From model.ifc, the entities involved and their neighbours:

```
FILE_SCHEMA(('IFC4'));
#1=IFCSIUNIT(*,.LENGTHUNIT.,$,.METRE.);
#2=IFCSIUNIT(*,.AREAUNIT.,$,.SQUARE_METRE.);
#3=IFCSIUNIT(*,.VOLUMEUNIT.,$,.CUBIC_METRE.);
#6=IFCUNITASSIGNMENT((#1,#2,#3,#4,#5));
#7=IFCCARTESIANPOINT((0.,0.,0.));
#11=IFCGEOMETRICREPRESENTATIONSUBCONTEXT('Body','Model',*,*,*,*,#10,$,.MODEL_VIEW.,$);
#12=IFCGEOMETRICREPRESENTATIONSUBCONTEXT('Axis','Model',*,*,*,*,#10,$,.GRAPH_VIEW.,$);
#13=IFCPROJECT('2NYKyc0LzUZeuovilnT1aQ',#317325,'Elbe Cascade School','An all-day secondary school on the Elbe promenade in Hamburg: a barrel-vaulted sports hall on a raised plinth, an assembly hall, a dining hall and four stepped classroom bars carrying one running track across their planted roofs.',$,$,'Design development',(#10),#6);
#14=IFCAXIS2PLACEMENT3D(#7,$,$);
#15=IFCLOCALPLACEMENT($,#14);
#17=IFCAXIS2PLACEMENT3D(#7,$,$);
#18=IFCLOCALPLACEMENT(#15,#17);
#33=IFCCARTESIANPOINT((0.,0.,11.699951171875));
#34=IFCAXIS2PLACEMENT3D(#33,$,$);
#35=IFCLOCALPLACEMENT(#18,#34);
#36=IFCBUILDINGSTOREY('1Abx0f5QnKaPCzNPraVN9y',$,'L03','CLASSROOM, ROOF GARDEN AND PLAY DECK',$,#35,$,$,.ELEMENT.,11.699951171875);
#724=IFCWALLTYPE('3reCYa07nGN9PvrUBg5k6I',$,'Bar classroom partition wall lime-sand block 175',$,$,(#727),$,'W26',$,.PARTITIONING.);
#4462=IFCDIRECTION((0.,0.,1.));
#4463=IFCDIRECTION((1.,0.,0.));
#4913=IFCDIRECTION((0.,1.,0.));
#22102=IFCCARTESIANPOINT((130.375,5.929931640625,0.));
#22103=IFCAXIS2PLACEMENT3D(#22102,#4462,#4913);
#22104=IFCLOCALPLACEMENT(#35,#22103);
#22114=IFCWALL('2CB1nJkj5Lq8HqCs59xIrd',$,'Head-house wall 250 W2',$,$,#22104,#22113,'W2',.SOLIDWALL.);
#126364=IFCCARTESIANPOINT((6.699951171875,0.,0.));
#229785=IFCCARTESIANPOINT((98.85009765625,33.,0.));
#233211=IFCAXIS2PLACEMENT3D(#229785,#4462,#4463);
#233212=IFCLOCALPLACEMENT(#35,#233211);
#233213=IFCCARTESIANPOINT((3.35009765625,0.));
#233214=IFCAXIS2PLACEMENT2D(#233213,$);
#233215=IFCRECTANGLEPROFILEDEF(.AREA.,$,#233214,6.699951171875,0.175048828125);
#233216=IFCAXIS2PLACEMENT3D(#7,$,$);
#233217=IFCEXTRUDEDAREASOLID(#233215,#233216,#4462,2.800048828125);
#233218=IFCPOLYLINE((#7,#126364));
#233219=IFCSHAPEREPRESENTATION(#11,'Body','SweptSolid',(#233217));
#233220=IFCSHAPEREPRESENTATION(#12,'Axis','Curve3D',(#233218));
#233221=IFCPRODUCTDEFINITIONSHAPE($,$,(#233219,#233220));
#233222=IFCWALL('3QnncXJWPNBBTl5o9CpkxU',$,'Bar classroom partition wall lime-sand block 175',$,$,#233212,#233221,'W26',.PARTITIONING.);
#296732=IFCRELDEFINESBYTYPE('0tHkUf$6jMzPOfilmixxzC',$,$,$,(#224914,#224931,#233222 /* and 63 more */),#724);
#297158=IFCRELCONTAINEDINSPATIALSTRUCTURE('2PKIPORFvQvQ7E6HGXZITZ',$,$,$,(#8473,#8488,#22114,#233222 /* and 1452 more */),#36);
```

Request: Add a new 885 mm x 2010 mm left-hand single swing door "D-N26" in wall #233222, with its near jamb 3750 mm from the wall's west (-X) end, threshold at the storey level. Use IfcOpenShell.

```python
import numpy as np
import ifcopenshell
import ifcopenshell.api.feature
import ifcopenshell.api.geometry
import ifcopenshell.api.root
import ifcopenshell.api.spatial
import ifcopenshell.geom
import ifcopenshell.util.element
import ifcopenshell.util.placement
import ifcopenshell.util.representation
import ifcopenshell.util.shape
import ifcopenshell.util.unit

model = ifcopenshell.open("model.ifc")
unit_scale = ifcopenshell.util.unit.calculate_unit_scale(model)
settings = ifcopenshell.geom.settings()


def volume(element):
    """Net volume in cubic metres, openings subtracted."""
    shape = ifcopenshell.geom.create_shape(settings, element)
    return ifcopenshell.util.shape.get_volume(shape.geometry)


wall = model.by_guid("3QnncXJWPNBBTl5o9CpkxU")
storey = ifcopenshell.util.element.get_container(wall, ifc_class="IfcBuildingStorey")
context = ifcopenshell.util.representation.get_context(model, "Model", "Body", "MODEL_VIEW")
before = volume(wall)

width, height, from_end, sill = 0.885, 2.01, 3.75, 0.0  # metres

# The wall runs along its own X axis, and the end named is its -X end.
wall_shape = ifcopenshell.geom.create_shape(settings, wall)
x, y, z = ifcopenshell.util.shape.get_vertices(wall_shape.geometry).T
start = x.min() + from_end
face, thickness = float(y.min()), float(y.max() - y.min())
wall_matrix = ifcopenshell.util.placement.get_local_placement(wall.ObjectPlacement)
level = ifcopenshell.util.placement.get_local_placement(storey.ObjectPlacement)[2, 3]


def in_wall(x, y):
    """Placement at x, y metres in the wall's axes, at sill height."""
    matrix = wall_matrix.copy()
    matrix[:, 3] = wall_matrix @ np.array([x / unit_scale, y / unit_scale, 0.0, 1.0])
    matrix[2, 3] = level + sill / unit_scale
    return matrix


# Opening: a box that overshoots both wall faces by 50 mm.
opening = ifcopenshell.api.root.create_entity(model, ifc_class="IfcOpeningElement", predefined_type="OPENING")
box = ifcopenshell.api.geometry.add_wall_representation(
    model, context=context, length=width, height=height, thickness=thickness + 0.1
)
ifcopenshell.api.geometry.assign_representation(model, product=opening, representation=box)
ifcopenshell.api.geometry.edit_object_placement(model, product=opening, matrix=in_wall(start, face - 0.05), is_si=False)
ifcopenshell.api.feature.add_feature(model, feature=opening, element=wall)

door = ifcopenshell.api.root.create_entity(model, ifc_class="IfcDoor", name="D-N26", predefined_type="DOOR")
door.OverallWidth, door.OverallHeight = width / unit_scale, height / unit_scale
door.OperationType = "SINGLE_SWING_LEFT"
body = ifcopenshell.api.geometry.add_door_representation(
    model,
    context=context,
    overall_width=door.OverallWidth,
    overall_height=door.OverallHeight,
    operation_type="SINGLE_SWING_LEFT",
    lining_properties={"LiningDepth": thickness / unit_scale, "ThresholdDepth": thickness / unit_scale},
)
ifcopenshell.api.geometry.assign_representation(model, product=door, representation=body)
ifcopenshell.api.spatial.assign_container(model, products=[door], relating_structure=storey)
ifcopenshell.api.feature.add_filling(model, opening=opening, element=door)

# The lining spans the wall, so the door starts at the wall face.
ifcopenshell.api.geometry.edit_object_placement(model, product=door, matrix=in_wall(start, face), is_si=False)

after = volume(wall)

print(f"wall volume {before:.3f} -> {after:.3f} m3")

model.write("model_rev.ifc")
```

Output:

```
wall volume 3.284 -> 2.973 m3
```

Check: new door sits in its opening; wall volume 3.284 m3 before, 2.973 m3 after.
